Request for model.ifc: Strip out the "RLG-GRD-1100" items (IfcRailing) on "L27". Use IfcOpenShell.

First a look at what the model holds.

```python
import ifcopenshell
import ifcopenshell.util.element

model = ifcopenshell.open("model.ifc")
print(model.schema)
storey = next(s for s in model.by_type("IfcBuildingStorey") if s.Name == "L27")
railings = [e for e in ifcopenshell.util.element.get_decomposition(storey) if e.is_a("IfcRailing")]
seen = {}
for e in railings:
    element_type = ifcopenshell.util.element.get_type(e)
    name = element_type.Name if element_type not in (None, e) else None
    seen[name] = seen.get(name, 0) + 1
for name, count in sorted(seen.items(), key=str):
    print(count, "x", name)
```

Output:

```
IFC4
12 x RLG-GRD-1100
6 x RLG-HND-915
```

```python
import ifcopenshell
import ifcopenshell.api.root
import ifcopenshell.util.element

model = ifcopenshell.open("model.ifc")

storey = next(s for s in model.by_type("IfcBuildingStorey") if s.Name == "L27")
railings = [e for e in ifcopenshell.util.element.get_decomposition(storey) if e.is_a("IfcRailing")]
targets = [e for e in railings if (t := ifcopenshell.util.element.get_type(e)) not in (None, e) and t.Name == "RLG-GRD-1100"]

for e in targets:
    ifcopenshell.api.root.remove_product(model, product=e)
print(len(targets), "removed")

model.write("model_rev.ifc")
```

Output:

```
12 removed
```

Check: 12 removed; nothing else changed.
